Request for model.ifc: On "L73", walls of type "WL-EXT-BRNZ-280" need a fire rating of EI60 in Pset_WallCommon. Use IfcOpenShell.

First a look at what the model holds.

```python
import ifcopenshell
import ifcopenshell.util.element

model = ifcopenshell.open("model.ifc")
print(model.schema)
storey = next(s for s in model.by_type("IfcBuildingStorey") if s.Name == "L73")
walls = [e for e in ifcopenshell.util.element.get_decomposition(storey) if e.is_a("IfcWall")]
seen = {}
for e in walls:
    element_type = ifcopenshell.util.element.get_type(e)
    key = (element_type.Name if element_type != e and element_type else None, ifcopenshell.util.element.get_pset(e, "Pset_WallCommon", "FireRating"))
    seen[key] = seen.get(key, 0) + 1
for (name, value), count in sorted(seen.items(), key=str):
    print(count, "x", name, "|", value)
```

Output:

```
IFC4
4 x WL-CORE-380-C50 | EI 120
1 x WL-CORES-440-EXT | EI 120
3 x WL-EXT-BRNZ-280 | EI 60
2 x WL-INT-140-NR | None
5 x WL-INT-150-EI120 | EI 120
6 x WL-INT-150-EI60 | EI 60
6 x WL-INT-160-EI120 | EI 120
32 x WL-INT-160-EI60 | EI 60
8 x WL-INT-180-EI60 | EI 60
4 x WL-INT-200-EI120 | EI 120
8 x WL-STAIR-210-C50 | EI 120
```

```python
import ifcopenshell
import ifcopenshell.api.pset
import ifcopenshell.util.element

model = ifcopenshell.open("model.ifc")

storey = next(s for s in model.by_type("IfcBuildingStorey") if s.Name == "L73")
walls = [e for e in ifcopenshell.util.element.get_decomposition(storey) if e.is_a("IfcWall")]

count = 0
for e in walls:
    element_type = ifcopenshell.util.element.get_type(e)
    if element_type in (None, e) or element_type.Name != "WL-EXT-BRNZ-280":
        continue
    found = ifcopenshell.util.element.get_pset(e, "Pset_WallCommon", should_inherit=False)
    if found:
        pset = model.by_id(found["id"])
        if len(ifcopenshell.util.element.get_elements_by_pset(pset)) > 1:
            pset = ifcopenshell.api.pset.unshare_pset(model, products=[e], pset=pset)[0]
    else:
        pset = ifcopenshell.api.pset.add_pset(model, product=e, name="Pset_WallCommon")
    ifcopenshell.api.pset.edit_pset(model, pset=pset, properties={"FireRating": "EI60"})
    count += 1

print(count, "walls updated")

model.write("model-out.ifc")
```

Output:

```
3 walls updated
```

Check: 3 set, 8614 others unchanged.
